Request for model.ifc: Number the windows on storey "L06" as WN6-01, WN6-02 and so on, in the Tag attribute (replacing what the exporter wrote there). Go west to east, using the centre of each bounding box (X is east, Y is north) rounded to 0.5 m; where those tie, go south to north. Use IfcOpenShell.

First a look at what the model holds.

```python
import ifcopenshell
import ifcopenshell.util.element
import ifcopenshell.util.placement

model = ifcopenshell.open("model.ifc")
print(model.schema)
storey = next(s for s in model.by_type("IfcBuildingStorey") if s.Name == "L06")
windows = [e for e in ifcopenshell.util.element.get_decomposition(storey) if e.is_a("IfcWindow")]
for e in sorted(windows, key=lambda e: e.id()):
    origin = ifcopenshell.util.placement.get_local_placement(e.ObjectPlacement)[:3, 3]
    print(e.id(), e.Tag, e.Name, origin.round(2) + 0.0, sep=" | ")
```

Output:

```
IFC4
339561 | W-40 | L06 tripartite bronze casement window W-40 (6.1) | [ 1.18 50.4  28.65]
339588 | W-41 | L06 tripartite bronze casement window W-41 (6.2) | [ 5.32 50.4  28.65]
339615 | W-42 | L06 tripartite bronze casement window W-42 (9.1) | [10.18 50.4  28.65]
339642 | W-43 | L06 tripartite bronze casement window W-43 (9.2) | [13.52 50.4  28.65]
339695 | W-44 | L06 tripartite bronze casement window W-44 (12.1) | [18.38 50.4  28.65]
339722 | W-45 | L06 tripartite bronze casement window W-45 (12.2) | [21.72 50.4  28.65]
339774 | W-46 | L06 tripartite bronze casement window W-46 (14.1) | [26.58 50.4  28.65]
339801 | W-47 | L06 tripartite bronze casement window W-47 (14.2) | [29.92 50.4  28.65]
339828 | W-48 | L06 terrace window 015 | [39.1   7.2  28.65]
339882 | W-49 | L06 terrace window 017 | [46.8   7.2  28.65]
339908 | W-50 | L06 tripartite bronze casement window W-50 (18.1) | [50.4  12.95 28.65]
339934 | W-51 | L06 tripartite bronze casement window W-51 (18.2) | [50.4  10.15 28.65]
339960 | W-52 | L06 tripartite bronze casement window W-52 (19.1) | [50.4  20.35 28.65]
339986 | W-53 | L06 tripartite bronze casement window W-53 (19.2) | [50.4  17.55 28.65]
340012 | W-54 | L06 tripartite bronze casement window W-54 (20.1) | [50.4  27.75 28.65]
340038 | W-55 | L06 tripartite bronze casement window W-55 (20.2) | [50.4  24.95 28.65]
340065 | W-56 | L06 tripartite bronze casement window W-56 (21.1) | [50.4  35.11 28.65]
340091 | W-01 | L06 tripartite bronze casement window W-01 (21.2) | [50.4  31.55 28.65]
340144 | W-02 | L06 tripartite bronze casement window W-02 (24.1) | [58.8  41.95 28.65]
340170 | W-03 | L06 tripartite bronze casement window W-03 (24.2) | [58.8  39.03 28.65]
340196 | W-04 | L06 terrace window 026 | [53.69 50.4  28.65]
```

```python
import ifcopenshell
import ifcopenshell.geom
import ifcopenshell.util.element
import ifcopenshell.util.shape

model = ifcopenshell.open("model.ifc")
settings = ifcopenshell.geom.settings()
settings.set("use-world-coords", True)


def centre(element):
    shape = ifcopenshell.geom.create_shape(settings, element)
    return ifcopenshell.util.shape.get_bbox_centroid(shape.geometry)


storey = next(s for s in model.by_type("IfcBuildingStorey") if s.Name == "L06")
windows = [e for e in ifcopenshell.util.element.get_decomposition(storey) if e.is_a("IfcWindow")]

# Insertion points can sit at a corner or the storey origin, so sort by the geometry (in metres).
centres = {e: centre(e) for e in windows}
windows.sort(key=lambda e: (round(centres[e][0] / 0.5), centres[e][1]))

for i, e in enumerate(windows, start=1):
    number = f"WN6-{i:02d}"
    e.Tag = number
    print(e.id(), number)

model.write("model_updated.ifc")
```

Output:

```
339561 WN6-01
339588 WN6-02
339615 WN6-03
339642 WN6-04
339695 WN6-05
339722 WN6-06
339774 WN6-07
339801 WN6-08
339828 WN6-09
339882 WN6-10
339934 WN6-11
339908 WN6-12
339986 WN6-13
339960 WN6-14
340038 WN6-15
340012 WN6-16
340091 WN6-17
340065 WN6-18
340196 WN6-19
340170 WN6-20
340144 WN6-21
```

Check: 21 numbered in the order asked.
